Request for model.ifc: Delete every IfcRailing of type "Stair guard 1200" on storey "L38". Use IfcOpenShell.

First a look at what the model holds.

```python
import ifcopenshell
import ifcopenshell.util.element

model = ifcopenshell.open("model.ifc")
print(model.schema)
storey = next(s for s in model.by_type("IfcBuildingStorey") if s.Name == "L38")
railings = [e for e in ifcopenshell.util.element.get_decomposition(storey) if e.is_a("IfcRailing")]
seen = {}
for e in railings:
    element_type = ifcopenshell.util.element.get_type(e)
    name = element_type.Name if element_type not in (None, e) else None
    seen[name] = seen.get(name, 0) + 1
for name, count in sorted(seen.items(), key=str):
    print(count, "x", name)
```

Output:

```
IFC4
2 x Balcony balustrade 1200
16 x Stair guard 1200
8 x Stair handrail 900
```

```python
import ifcopenshell
import ifcopenshell.api.root
import ifcopenshell.util.element

model = ifcopenshell.open("model.ifc")

storey = next(s for s in model.by_type("IfcBuildingStorey") if s.Name == "L38")
railings = [e for e in ifcopenshell.util.element.get_decomposition(storey) if e.is_a("IfcRailing")]
targets = [e for e in railings if (t := ifcopenshell.util.element.get_type(e)) not in (None, e) and t.Name == "Stair guard 1200"]

for e in targets:
    ifcopenshell.api.root.remove_product(model, product=e)
print(len(targets), "removed")

model.write("model-out.ifc")
```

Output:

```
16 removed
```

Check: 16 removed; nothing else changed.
